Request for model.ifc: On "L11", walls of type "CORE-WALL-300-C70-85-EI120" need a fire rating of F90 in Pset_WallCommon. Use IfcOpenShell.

First a look at what the model holds.

```python
import ifcopenshell
import ifcopenshell.util.element

model = ifcopenshell.open("model.ifc")
print(model.schema)
storey = next(s for s in model.by_type("IfcBuildingStorey") if s.Name == "L11")
walls = [e for e in ifcopenshell.util.element.get_decomposition(storey) if e.is_a("IfcWall")]
seen = {}
for e in walls:
    element_type = ifcopenshell.util.element.get_type(e)
    key = (element_type.Name if element_type != e and element_type else None, ifcopenshell.util.element.get_pset(e, "Pset_WallCommon", "FireRating"))
    seen[key] = seen.get(key, 0) + 1
for (name, value), count in sorted(seen.items(), key=str):
    print(count, "x", name, "|", value)
```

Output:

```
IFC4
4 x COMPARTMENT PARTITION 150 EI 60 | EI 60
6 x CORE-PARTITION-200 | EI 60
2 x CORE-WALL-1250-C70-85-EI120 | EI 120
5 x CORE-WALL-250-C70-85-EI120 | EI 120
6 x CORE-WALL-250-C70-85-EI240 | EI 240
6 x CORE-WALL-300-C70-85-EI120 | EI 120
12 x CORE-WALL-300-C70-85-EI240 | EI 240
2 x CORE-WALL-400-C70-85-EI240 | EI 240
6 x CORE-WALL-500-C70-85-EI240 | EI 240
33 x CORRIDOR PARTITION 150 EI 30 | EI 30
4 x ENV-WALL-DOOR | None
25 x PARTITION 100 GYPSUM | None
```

```python
import ifcopenshell
import ifcopenshell.api.pset
import ifcopenshell.util.element

model = ifcopenshell.open("model.ifc")

storey = next(s for s in model.by_type("IfcBuildingStorey") if s.Name == "L11")
walls = [e for e in ifcopenshell.util.element.get_decomposition(storey) if e.is_a("IfcWall")]

count = 0
for e in walls:
    element_type = ifcopenshell.util.element.get_type(e)
    if element_type in (None, e) or element_type.Name != "CORE-WALL-300-C70-85-EI120":
        continue
    found = ifcopenshell.util.element.get_pset(e, "Pset_WallCommon", should_inherit=False)
    if found:
        pset = model.by_id(found["id"])
        if len(ifcopenshell.util.element.get_elements_by_pset(pset)) > 1:
            pset = ifcopenshell.api.pset.unshare_pset(model, products=[e], pset=pset)[0]
    else:
        pset = ifcopenshell.api.pset.add_pset(model, product=e, name="Pset_WallCommon")
    ifcopenshell.api.pset.edit_pset(model, pset=pset, properties={"FireRating": "F90"})
    count += 1

print(count, "walls updated")

model.write("model_rev.ifc")
```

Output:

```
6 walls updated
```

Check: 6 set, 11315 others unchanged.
